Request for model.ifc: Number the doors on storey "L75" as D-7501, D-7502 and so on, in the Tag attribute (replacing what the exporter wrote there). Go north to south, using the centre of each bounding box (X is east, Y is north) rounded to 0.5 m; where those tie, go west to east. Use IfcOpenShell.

First a look at what the model holds.

```python
import ifcopenshell
import ifcopenshell.util.element
import ifcopenshell.util.placement

model = ifcopenshell.open("model.ifc")
print(model.schema)
storey = next(s for s in model.by_type("IfcBuildingStorey") if s.Name == "L75")
doors = [e for e in ifcopenshell.util.element.get_decomposition(storey) if e.is_a("IfcDoor")]
for e in sorted(doors, key=lambda e: e.id()):
    origin = ifcopenshell.util.placement.get_local_placement(e.ObjectPlacement)[:3, 3]
    print(e.id(), e.Tag, e.Name, origin.round(2) + 0.0, sep=" | ")
```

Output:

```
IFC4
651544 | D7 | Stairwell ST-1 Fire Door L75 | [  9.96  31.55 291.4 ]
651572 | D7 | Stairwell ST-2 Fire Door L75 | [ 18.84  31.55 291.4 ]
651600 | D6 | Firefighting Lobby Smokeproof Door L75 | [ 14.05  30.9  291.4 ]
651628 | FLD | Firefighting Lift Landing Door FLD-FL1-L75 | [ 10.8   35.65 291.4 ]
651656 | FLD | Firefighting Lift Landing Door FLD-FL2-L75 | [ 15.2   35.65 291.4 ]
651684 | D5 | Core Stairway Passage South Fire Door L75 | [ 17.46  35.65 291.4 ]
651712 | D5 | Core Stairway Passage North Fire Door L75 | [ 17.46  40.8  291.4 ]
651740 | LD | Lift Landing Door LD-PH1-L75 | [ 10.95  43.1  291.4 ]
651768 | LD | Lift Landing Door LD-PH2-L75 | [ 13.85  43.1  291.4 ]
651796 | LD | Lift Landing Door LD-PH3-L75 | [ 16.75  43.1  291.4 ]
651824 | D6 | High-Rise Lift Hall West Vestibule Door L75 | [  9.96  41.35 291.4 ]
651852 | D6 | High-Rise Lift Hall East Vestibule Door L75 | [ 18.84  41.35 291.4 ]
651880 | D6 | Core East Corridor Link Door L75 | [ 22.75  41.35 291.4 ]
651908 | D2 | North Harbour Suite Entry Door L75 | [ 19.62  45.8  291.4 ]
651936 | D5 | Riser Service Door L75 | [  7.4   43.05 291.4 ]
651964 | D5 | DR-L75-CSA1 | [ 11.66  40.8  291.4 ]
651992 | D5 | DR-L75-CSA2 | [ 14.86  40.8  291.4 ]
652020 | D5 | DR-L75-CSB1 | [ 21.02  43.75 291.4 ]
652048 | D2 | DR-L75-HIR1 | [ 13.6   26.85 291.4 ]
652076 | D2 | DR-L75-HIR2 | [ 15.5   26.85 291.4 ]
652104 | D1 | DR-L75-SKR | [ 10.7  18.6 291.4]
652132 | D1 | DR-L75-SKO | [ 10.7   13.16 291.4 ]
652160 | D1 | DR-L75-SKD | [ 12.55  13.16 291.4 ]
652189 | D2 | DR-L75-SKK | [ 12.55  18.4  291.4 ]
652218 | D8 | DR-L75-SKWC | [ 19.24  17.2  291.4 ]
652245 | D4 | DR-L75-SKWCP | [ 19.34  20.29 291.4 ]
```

```python
import ifcopenshell
import ifcopenshell.geom
import ifcopenshell.util.element
import ifcopenshell.util.shape

model = ifcopenshell.open("model.ifc")
settings = ifcopenshell.geom.settings()
settings.set("use-world-coords", True)


def centre(element):
    shape = ifcopenshell.geom.create_shape(settings, element)
    return ifcopenshell.util.shape.get_bbox_centroid(shape.geometry)


storey = next(s for s in model.by_type("IfcBuildingStorey") if s.Name == "L75")
doors = [e for e in ifcopenshell.util.element.get_decomposition(storey) if e.is_a("IfcDoor")]

# Insertion points can sit at a corner or the storey origin, so sort by the geometry (in metres).
centres = {e: centre(e) for e in doors}
doors.sort(key=lambda e: (-round(centres[e][1] / 0.5), centres[e][0]))

for i, e in enumerate(doors, start=1):
    number = f"D-75{i:02d}"
    e.Tag = number
    print(e.id(), number)

model.write("model_v2.ifc")
```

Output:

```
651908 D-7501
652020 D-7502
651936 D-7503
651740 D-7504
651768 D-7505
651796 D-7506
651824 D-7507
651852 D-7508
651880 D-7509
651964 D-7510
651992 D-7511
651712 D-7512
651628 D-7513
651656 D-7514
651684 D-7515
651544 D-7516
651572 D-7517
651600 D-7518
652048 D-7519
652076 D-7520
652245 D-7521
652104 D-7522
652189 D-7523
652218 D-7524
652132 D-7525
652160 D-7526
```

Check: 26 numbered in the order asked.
